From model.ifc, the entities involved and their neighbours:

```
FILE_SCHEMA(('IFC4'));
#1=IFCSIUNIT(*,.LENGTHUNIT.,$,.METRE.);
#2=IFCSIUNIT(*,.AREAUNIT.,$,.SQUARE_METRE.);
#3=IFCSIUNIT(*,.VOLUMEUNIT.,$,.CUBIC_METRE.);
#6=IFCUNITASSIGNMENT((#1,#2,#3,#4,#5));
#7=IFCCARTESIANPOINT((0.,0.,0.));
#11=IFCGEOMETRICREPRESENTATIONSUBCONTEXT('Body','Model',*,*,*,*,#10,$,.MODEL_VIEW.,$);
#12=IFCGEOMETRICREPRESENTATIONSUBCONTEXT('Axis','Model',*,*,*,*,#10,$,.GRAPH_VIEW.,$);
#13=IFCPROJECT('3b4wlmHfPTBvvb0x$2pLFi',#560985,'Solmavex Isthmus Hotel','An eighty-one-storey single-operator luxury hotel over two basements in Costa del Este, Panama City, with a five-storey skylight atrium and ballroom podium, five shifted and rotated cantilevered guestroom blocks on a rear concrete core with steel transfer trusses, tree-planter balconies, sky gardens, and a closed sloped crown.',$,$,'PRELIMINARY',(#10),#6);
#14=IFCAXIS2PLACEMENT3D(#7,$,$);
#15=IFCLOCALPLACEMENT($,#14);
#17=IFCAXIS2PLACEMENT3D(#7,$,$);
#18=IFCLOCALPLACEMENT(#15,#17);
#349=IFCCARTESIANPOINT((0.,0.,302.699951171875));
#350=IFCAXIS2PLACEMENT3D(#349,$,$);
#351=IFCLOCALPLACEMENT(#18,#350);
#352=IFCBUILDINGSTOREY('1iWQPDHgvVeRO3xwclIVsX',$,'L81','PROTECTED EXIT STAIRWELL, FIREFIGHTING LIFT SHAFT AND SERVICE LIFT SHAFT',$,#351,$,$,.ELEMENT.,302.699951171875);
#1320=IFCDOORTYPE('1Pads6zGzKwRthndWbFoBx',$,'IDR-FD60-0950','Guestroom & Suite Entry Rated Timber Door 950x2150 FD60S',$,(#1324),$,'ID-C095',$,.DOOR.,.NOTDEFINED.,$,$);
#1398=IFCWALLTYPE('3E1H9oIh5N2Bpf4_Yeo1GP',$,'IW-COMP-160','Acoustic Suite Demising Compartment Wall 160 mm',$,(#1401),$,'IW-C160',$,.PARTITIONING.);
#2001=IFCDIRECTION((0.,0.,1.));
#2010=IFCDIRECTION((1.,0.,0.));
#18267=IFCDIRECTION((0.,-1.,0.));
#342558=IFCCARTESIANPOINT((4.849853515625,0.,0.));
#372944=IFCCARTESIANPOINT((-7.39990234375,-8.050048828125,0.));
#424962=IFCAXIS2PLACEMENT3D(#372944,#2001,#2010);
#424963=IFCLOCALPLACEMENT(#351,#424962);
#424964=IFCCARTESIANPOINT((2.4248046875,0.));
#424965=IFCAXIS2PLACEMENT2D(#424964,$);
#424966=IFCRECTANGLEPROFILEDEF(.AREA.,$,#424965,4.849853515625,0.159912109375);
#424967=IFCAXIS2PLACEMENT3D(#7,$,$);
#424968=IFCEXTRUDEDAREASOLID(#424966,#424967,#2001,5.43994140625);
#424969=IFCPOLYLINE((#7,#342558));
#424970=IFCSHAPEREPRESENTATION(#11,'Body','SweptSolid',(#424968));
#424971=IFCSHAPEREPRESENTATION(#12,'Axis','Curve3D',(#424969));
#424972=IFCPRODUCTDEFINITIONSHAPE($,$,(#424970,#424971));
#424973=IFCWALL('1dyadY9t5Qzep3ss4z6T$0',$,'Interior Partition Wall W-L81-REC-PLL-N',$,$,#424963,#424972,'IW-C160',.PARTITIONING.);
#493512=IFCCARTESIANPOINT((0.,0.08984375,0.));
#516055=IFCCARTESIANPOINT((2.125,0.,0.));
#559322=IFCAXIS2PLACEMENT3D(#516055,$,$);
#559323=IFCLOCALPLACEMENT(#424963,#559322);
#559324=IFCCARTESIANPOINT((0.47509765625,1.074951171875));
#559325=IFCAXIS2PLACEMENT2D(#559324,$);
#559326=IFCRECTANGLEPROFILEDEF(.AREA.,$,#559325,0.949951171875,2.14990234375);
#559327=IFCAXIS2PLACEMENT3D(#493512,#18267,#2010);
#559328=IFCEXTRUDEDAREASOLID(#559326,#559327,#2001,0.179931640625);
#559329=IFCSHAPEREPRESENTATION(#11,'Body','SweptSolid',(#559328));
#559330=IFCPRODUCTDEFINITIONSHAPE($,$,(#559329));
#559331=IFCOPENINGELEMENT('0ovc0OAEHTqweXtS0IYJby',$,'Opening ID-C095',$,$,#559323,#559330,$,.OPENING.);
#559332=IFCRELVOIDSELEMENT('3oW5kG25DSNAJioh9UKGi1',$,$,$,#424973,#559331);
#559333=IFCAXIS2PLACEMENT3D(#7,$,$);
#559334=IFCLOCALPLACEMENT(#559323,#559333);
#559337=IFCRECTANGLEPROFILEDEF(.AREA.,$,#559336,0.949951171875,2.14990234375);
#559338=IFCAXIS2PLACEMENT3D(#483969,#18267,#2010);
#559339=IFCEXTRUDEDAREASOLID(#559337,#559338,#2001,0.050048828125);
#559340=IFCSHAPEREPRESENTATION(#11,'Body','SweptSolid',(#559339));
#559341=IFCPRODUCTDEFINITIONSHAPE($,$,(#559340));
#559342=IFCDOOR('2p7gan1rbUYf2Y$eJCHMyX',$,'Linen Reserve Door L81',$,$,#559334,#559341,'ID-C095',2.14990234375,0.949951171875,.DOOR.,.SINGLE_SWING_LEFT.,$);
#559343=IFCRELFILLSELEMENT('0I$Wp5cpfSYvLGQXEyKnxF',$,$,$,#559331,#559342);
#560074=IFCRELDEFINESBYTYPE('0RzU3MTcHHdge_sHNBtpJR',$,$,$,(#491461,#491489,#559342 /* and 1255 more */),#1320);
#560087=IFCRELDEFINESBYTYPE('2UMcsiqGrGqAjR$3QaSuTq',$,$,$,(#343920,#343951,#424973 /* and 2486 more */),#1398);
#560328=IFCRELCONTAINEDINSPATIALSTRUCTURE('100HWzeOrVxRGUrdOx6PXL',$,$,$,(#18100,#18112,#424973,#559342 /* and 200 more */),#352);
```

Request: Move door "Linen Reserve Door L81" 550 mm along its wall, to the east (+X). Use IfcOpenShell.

```python
import ifcopenshell
import ifcopenshell.api.geometry
import ifcopenshell.util.placement
import ifcopenshell.util.unit

model = ifcopenshell.open("model.ifc")
unit_scale = ifcopenshell.util.unit.calculate_unit_scale(model)

door = model.by_guid("2p7gan1rbUYf2Y$eJCHMyX")
opening = door.FillsVoids[0].RelatingOpeningElement
wall = opening.VoidsElements[0].RelatingBuildingElement

wall_matrix = ifcopenshell.util.placement.get_local_placement(wall.ObjectPlacement)
shift = wall_matrix[:3, 0] * 0.55 / unit_scale
before = ifcopenshell.util.placement.get_local_placement(door.ObjectPlacement)[:3, 3].copy()

# The door is placed relative to its opening, so it follows when the opening moves.
matrix = ifcopenshell.util.placement.get_local_placement(opening.ObjectPlacement)
matrix[:3, 3] += shift
ifcopenshell.api.geometry.edit_object_placement(
    model, product=opening, matrix=matrix, is_si=False, should_transform_children=True
)

after = ifcopenshell.util.placement.get_local_placement(door.ObjectPlacement)[:3, 3]
print("door moved by", (after - before).round(3) + 0.0)

model.write("model_v2.ifc")
```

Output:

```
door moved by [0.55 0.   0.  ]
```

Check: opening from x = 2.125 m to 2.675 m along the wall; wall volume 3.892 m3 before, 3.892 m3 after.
